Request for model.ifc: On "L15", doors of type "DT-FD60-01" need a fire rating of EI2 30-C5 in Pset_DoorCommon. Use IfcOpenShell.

First a look at what the model holds.

```python
import ifcopenshell
import ifcopenshell.util.element

model = ifcopenshell.open("model.ifc")
print(model.schema)
storey = next(s for s in model.by_type("IfcBuildingStorey") if s.Name == "L15")
doors = [e for e in ifcopenshell.util.element.get_decomposition(storey) if e.is_a("IfcDoor")]
seen = {}
for e in doors:
    element_type = ifcopenshell.util.element.get_type(e)
    key = (element_type.Name if element_type != e and element_type else None, ifcopenshell.util.element.get_pset(e, "Pset_DoorCommon", "FireRating"))
    seen[key] = seen.get(key, 0) + 1
for (name, value), count in sorted(seen.items(), key=str):
    print(count, "x", name, "|", value)
```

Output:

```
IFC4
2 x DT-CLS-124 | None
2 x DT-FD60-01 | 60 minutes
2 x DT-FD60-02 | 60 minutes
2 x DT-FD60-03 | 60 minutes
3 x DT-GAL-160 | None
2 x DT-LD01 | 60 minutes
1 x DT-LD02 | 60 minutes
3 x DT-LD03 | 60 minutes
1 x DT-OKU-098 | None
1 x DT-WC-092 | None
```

```python
import ifcopenshell
import ifcopenshell.api.pset
import ifcopenshell.util.element

model = ifcopenshell.open("model.ifc")

storey = next(s for s in model.by_type("IfcBuildingStorey") if s.Name == "L15")
doors = [e for e in ifcopenshell.util.element.get_decomposition(storey) if e.is_a("IfcDoor")]

count = 0
for e in doors:
    element_type = ifcopenshell.util.element.get_type(e)
    if element_type in (None, e) or element_type.Name != "DT-FD60-01":
        continue
    # add_pset returns the element's existing set when there is one.
    pset = ifcopenshell.api.pset.add_pset(model, product=e, name="Pset_DoorCommon")
    ifcopenshell.api.pset.edit_pset(model, pset=pset, properties={"FireRating": "EI2 30-C5"})
    count += 1

print(count, "doors updated")

model.write("model_edited.ifc")
```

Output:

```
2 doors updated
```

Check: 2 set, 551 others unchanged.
